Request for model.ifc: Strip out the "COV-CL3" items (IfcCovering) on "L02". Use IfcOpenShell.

First a look at what the model holds.

```python
import ifcopenshell
import ifcopenshell.util.element

model = ifcopenshell.open("model.ifc")
print(model.schema)
storey = next(s for s in model.by_type("IfcBuildingStorey") if s.Name == "L02")
coverings = [e for e in ifcopenshell.util.element.get_decomposition(storey) if e.is_a("IfcCovering")]
seen = {}
for e in coverings:
    element_type = ifcopenshell.util.element.get_type(e)
    name = element_type.Name if element_type not in (None, e) else None
    seen[name] = seen.get(name, 0) + 1
for name, count in sorted(seen.items(), key=str):
    print(count, "x", name)
```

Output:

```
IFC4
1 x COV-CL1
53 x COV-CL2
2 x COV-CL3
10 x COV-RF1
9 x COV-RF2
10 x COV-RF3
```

```python
import ifcopenshell
import ifcopenshell.api.root
import ifcopenshell.util.element

model = ifcopenshell.open("model.ifc")

storey = next(s for s in model.by_type("IfcBuildingStorey") if s.Name == "L02")
coverings = [e for e in ifcopenshell.util.element.get_decomposition(storey) if e.is_a("IfcCovering")]
targets = [e for e in coverings if (t := ifcopenshell.util.element.get_type(e)) not in (None, e) and t.Name == "COV-CL3"]

for e in targets:
    ifcopenshell.api.root.remove_product(model, product=e)
print(len(targets), "removed")

model.write("model_edited.ifc")
```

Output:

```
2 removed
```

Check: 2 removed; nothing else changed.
